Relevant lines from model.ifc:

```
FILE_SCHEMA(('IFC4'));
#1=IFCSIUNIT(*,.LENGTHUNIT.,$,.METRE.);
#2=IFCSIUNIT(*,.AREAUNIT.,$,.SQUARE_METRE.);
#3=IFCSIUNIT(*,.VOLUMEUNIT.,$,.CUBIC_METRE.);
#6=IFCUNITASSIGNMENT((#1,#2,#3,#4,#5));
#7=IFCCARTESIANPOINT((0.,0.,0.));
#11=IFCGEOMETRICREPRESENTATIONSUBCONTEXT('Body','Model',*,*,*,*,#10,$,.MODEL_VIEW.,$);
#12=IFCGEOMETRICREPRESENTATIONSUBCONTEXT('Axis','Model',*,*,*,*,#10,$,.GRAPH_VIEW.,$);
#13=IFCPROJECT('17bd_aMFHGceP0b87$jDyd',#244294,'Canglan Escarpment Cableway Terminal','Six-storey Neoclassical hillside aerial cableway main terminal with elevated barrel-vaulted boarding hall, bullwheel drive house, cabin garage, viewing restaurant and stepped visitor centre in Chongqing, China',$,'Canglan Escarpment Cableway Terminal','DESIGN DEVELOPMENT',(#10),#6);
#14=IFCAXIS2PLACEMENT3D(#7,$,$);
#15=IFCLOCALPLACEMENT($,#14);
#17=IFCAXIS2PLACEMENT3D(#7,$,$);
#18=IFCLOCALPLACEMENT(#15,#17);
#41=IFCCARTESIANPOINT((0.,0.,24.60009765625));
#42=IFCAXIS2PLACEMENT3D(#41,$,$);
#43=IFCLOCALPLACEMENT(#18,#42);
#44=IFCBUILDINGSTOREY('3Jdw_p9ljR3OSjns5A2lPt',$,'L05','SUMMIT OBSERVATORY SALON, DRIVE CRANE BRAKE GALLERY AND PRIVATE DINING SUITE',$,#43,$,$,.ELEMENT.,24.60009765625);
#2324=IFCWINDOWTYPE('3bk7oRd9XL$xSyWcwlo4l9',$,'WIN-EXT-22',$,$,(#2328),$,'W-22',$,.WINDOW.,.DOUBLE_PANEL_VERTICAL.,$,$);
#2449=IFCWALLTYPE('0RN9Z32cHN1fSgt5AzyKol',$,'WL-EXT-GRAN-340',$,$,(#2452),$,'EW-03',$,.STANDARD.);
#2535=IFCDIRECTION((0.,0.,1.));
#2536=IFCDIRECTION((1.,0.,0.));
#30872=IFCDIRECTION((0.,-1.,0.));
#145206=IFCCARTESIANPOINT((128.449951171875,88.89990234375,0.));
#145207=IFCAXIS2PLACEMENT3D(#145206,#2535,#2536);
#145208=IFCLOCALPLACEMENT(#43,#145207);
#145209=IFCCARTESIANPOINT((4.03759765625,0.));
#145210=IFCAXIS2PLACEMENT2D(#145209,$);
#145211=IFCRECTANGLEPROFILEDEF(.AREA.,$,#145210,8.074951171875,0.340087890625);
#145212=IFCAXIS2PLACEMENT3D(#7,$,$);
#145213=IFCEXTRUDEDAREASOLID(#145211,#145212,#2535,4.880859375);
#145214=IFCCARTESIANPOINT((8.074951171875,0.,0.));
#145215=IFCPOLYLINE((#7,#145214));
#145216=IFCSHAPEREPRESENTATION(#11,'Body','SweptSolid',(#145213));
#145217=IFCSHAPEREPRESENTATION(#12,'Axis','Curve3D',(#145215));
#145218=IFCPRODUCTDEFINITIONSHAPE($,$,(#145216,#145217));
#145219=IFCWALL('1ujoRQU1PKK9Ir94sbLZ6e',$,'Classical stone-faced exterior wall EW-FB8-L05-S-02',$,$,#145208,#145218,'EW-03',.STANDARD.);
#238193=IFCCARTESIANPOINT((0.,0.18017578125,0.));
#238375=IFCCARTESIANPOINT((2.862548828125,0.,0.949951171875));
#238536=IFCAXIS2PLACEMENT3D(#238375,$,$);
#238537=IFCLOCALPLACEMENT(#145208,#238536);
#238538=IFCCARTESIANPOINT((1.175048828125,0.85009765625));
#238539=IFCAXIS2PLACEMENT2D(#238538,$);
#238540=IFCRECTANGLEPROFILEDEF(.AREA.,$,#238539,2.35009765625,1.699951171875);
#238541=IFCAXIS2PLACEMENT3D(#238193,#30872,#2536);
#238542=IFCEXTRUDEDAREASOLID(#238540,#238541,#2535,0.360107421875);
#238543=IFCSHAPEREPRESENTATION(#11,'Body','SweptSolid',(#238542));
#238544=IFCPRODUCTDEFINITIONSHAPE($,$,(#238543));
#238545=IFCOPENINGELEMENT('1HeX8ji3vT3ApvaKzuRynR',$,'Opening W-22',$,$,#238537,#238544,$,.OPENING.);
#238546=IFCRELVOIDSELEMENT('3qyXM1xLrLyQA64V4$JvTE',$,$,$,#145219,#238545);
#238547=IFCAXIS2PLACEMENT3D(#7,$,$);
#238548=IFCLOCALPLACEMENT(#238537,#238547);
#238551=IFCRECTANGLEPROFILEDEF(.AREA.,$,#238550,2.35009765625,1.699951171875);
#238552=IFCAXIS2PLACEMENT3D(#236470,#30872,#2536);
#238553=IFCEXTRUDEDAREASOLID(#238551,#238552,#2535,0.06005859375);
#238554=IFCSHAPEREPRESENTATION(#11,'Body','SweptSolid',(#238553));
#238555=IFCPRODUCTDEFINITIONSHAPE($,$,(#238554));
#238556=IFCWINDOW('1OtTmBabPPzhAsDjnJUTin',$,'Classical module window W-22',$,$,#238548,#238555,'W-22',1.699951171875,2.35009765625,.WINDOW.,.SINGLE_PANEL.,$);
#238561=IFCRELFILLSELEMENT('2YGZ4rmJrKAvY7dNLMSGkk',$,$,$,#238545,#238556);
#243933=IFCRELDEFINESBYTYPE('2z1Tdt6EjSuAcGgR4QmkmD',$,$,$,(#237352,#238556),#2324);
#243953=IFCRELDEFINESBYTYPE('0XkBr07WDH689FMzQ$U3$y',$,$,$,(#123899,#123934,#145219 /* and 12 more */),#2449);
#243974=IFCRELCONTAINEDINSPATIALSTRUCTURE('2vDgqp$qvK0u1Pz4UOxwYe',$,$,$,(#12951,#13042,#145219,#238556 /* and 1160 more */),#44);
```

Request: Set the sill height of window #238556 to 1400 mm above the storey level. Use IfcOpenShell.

```python
import numpy as np
import ifcopenshell
import ifcopenshell.api.geometry
import ifcopenshell.geom
import ifcopenshell.util.element
import ifcopenshell.util.placement
import ifcopenshell.util.shape
import ifcopenshell.util.unit

model = ifcopenshell.open("model.ifc")
unit_scale = ifcopenshell.util.unit.calculate_unit_scale(model)

window = model.by_id(238556)
opening = window.FillsVoids[0].RelatingOpeningElement
storey = ifcopenshell.util.element.get_container(window, ifc_class="IfcBuildingStorey")
level = ifcopenshell.util.placement.get_local_placement(storey.ObjectPlacement)[2, 3]

# The opening's origin need not be at the sill, so measure its lowest point.
shape = ifcopenshell.geom.create_shape(ifcopenshell.geom.settings(), opening)
bottom = ifcopenshell.util.shape.get_shape_bottom_elevation(shape, shape.geometry) / unit_scale
dz = level + 1.4 - bottom

shift = np.array([0.0, 0.0, dz])
# The window is placed relative to its opening, so it follows when the opening moves.
matrix = ifcopenshell.util.placement.get_local_placement(opening.ObjectPlacement)
matrix[:3, 3] += shift
ifcopenshell.api.geometry.edit_object_placement(
    model, product=opening, matrix=matrix, is_si=False, should_transform_children=True
)

print(f"moved by {dz * unit_scale:+.3f} m")

model.write("model_rev.ifc")
```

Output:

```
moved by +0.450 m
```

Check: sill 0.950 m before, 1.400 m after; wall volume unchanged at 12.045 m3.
